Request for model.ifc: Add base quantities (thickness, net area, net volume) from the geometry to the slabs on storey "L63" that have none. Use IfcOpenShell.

First a look at what the model holds.

```python
import ifcopenshell
import ifcopenshell.util.element
import ifcopenshell.util.unit

model = ifcopenshell.open("model.ifc")
print(model.schema)
for unit_type in ("LENGTHUNIT", "AREAUNIT", "VOLUMEUNIT"):
    print(unit_type, ifcopenshell.util.unit.calculate_unit_scale(model, unit_type))
storey = next(s for s in model.by_type("IfcBuildingStorey") if s.Name == "L63")
slabs = [e for e in ifcopenshell.util.element.get_decomposition(storey) if e.is_a("IfcSlab")]
for e in sorted(slabs, key=lambda e: e.id()):
    print(e.id(), e.is_a(), e.Name, list(ifcopenshell.util.element.get_psets(e, qtos_only=True)), sep=" | ")
```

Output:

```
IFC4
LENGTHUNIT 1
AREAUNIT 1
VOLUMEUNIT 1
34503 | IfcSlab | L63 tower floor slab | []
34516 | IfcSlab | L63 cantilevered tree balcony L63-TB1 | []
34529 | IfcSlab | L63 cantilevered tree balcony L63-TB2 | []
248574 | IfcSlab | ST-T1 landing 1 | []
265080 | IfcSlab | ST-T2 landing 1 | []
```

```python
import ifcopenshell
import ifcopenshell.api.pset
import ifcopenshell.geom
import ifcopenshell.util.element
import ifcopenshell.util.shape
import ifcopenshell.util.unit

model = ifcopenshell.open("model.ifc")
unit_scale = ifcopenshell.util.unit.calculate_unit_scale(model)
area_scale = ifcopenshell.util.unit.calculate_unit_scale(model, "AREAUNIT")
volume_scale = ifcopenshell.util.unit.calculate_unit_scale(model, "VOLUMEUNIT")
settings = ifcopenshell.geom.settings()

storey = next(s for s in model.by_type("IfcBuildingStorey") if s.Name == "L63")
slabs = [e for e in ifcopenshell.util.element.get_decomposition(storey) if e.is_a("IfcSlab")]

for e in sorted(slabs, key=lambda e: e.id()):
    if ifcopenshell.util.element.get_psets(e, qtos_only=True, should_inherit=False):
        continue
    # Geometry comes back in metres, in the element's own axes.
    shape = ifcopenshell.geom.create_shape(settings, e)
    values = {
        "Width": ifcopenshell.util.shape.get_z(shape.geometry) / unit_scale,
        "NetArea": ifcopenshell.util.shape.get_footprint_area(shape.geometry) / area_scale,
        "NetVolume": ifcopenshell.util.shape.get_volume(shape.geometry) / volume_scale,
    }
    qto = ifcopenshell.api.pset.add_qto(model, product=e, name="Qto_SlabBaseQuantities")
    ifcopenshell.api.pset.edit_qto(model, qto=qto, properties=values)
    print(e.id(), {k: round(v, 3) for k, v in values.items()})

model.write("model_edited.ifc")
```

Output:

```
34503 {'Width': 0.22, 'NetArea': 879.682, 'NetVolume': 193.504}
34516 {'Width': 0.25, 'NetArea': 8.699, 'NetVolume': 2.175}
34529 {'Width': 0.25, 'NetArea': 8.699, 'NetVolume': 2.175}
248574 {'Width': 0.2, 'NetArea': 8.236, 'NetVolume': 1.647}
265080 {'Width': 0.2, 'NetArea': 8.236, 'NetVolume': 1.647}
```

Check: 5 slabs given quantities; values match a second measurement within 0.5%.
